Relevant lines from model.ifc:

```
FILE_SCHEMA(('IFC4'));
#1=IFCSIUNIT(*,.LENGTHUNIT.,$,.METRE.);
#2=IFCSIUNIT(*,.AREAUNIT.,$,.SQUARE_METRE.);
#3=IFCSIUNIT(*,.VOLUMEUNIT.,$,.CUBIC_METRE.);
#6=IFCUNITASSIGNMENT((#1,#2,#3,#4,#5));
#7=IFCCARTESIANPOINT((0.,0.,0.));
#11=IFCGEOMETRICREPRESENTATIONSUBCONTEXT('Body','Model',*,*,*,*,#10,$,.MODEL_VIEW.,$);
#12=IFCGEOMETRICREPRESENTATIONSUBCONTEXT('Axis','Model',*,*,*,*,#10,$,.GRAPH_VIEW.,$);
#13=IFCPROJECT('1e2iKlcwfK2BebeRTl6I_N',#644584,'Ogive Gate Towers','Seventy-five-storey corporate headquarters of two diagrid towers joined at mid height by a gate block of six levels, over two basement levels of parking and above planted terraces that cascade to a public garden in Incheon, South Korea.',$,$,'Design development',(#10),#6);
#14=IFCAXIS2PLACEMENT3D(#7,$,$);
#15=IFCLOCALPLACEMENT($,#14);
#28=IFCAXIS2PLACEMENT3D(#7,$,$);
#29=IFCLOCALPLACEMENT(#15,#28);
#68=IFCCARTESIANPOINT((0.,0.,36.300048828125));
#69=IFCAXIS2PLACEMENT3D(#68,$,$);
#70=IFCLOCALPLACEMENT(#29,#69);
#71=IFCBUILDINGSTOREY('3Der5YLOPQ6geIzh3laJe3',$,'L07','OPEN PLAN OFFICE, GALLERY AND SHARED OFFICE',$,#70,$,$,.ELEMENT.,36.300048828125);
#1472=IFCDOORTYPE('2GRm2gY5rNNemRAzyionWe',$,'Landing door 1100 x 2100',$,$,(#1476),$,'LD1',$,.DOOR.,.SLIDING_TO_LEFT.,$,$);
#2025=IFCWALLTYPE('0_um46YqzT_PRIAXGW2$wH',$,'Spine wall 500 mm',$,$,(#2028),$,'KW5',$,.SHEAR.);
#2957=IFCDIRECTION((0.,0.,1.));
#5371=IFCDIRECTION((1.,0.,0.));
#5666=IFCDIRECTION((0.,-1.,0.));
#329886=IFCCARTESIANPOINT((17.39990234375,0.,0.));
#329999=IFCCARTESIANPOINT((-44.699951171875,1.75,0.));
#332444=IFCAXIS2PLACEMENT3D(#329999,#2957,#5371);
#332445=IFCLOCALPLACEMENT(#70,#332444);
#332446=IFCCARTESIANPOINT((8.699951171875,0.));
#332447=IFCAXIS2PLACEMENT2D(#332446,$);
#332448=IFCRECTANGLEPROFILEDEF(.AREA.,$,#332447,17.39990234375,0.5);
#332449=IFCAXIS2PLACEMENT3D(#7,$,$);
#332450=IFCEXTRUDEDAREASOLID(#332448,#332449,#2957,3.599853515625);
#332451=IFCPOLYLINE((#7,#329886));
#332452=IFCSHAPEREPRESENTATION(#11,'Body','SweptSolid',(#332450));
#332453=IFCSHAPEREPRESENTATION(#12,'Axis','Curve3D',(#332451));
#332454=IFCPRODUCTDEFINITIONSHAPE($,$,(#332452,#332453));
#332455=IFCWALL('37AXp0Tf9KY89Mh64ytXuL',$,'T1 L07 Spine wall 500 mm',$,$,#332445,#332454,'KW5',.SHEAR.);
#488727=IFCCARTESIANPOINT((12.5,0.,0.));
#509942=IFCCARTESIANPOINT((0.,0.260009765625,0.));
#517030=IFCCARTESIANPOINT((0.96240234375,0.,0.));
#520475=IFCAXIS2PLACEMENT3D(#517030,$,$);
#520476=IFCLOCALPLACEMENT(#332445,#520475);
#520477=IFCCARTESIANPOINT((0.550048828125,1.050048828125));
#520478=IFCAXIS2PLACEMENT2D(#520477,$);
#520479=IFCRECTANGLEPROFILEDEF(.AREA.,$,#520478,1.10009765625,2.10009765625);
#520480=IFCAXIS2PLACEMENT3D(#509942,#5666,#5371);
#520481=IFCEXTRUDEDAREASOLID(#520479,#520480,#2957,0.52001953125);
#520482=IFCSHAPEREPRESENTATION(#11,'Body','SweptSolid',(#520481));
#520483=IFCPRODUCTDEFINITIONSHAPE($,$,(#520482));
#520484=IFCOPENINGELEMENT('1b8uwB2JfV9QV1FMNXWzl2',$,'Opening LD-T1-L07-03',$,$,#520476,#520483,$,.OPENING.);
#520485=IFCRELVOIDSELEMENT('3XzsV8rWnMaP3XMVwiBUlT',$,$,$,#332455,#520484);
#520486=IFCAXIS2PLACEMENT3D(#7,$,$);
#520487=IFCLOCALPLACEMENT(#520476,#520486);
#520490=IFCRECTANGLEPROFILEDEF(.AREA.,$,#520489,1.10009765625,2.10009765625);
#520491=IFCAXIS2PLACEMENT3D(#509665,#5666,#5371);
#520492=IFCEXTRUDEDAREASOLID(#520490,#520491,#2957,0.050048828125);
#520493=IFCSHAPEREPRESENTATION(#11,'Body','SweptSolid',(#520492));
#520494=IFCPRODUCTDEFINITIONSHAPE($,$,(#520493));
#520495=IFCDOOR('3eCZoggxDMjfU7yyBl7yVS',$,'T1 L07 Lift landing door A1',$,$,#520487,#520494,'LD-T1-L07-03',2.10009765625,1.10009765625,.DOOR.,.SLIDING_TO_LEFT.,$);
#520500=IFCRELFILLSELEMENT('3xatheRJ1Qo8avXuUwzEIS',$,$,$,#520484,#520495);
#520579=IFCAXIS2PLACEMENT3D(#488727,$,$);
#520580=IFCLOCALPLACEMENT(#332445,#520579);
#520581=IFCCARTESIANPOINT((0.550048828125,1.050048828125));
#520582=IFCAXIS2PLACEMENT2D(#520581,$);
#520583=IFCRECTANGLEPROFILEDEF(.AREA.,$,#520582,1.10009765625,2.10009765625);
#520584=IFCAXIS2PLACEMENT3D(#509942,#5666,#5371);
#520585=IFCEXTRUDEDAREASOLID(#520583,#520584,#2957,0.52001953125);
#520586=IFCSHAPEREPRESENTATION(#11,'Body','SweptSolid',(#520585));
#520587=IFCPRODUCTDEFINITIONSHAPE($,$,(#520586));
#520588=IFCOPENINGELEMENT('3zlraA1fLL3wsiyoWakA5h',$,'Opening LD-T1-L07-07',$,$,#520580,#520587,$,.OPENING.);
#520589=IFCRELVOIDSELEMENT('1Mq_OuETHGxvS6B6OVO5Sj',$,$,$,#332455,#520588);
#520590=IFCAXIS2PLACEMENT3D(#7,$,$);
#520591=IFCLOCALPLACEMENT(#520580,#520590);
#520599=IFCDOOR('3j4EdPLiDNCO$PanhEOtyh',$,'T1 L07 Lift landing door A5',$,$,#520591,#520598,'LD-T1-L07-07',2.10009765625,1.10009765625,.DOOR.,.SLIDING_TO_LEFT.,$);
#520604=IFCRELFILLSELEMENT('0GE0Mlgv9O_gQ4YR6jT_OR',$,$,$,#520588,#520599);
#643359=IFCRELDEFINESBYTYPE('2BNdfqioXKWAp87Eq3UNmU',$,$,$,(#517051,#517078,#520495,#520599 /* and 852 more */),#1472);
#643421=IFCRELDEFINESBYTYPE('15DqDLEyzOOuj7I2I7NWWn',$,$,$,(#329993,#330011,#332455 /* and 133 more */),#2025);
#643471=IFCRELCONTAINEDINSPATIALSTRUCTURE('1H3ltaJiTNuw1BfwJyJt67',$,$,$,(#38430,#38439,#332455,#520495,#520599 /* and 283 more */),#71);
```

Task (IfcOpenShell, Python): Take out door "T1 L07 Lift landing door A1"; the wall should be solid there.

```python
import ifcopenshell
import ifcopenshell.api.feature
import ifcopenshell.api.root
import ifcopenshell.geom
import ifcopenshell.util.shape

model = ifcopenshell.open("model.ifc")
settings = ifcopenshell.geom.settings()


def volume(element):
    """Net volume in cubic metres, openings subtracted."""
    shape = ifcopenshell.geom.create_shape(settings, element)
    return ifcopenshell.util.shape.get_volume(shape.geometry)


door = model.by_id(520495)
opening = door.FillsVoids[0].RelatingOpeningElement
wall = opening.VoidsElements[0].RelatingBuildingElement
before = volume(wall)

ifcopenshell.api.root.remove_product(model, product=door)
ifcopenshell.api.feature.remove_feature(model, feature=opening)

after = volume(wall)

print(f"wall volume {before:.3f} -> {after:.3f} m3")

model.write("model_edited.ifc")
```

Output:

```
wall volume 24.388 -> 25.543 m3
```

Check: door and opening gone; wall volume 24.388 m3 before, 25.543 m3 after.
